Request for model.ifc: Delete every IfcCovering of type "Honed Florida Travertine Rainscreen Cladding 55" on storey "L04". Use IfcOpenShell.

First a look at what the model holds.

```python
import ifcopenshell
import ifcopenshell.util.element

model = ifcopenshell.open("model.ifc")
print(model.schema)
storey = next(s for s in model.by_type("IfcBuildingStorey") if s.Name == "L04")
coverings = [e for e in ifcopenshell.util.element.get_decomposition(storey) if e.is_a("IfcCovering")]
seen = {}
for e in coverings:
    element_type = ifcopenshell.util.element.get_type(e)
    name = element_type.Name if element_type not in (None, e) else None
    seen[name] = seen.get(name, 0) + 1
for name, count in sorted(seen.items(), key=str):
    print(count, "x", name)
```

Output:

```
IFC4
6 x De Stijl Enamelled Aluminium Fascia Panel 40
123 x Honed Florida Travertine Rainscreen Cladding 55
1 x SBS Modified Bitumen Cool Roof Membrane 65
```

```python
import ifcopenshell
import ifcopenshell.api.root
import ifcopenshell.util.element

model = ifcopenshell.open("model.ifc")

storey = next(s for s in model.by_type("IfcBuildingStorey") if s.Name == "L04")
coverings = [e for e in ifcopenshell.util.element.get_decomposition(storey) if e.is_a("IfcCovering")]
targets = [e for e in coverings if (t := ifcopenshell.util.element.get_type(e)) not in (None, e) and t.Name == "Honed Florida Travertine Rainscreen Cladding 55"]

for e in targets:
    ifcopenshell.api.root.remove_product(model, product=e)
print(len(targets), "removed")

model.write("model_edited.ifc")
```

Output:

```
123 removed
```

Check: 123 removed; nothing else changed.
